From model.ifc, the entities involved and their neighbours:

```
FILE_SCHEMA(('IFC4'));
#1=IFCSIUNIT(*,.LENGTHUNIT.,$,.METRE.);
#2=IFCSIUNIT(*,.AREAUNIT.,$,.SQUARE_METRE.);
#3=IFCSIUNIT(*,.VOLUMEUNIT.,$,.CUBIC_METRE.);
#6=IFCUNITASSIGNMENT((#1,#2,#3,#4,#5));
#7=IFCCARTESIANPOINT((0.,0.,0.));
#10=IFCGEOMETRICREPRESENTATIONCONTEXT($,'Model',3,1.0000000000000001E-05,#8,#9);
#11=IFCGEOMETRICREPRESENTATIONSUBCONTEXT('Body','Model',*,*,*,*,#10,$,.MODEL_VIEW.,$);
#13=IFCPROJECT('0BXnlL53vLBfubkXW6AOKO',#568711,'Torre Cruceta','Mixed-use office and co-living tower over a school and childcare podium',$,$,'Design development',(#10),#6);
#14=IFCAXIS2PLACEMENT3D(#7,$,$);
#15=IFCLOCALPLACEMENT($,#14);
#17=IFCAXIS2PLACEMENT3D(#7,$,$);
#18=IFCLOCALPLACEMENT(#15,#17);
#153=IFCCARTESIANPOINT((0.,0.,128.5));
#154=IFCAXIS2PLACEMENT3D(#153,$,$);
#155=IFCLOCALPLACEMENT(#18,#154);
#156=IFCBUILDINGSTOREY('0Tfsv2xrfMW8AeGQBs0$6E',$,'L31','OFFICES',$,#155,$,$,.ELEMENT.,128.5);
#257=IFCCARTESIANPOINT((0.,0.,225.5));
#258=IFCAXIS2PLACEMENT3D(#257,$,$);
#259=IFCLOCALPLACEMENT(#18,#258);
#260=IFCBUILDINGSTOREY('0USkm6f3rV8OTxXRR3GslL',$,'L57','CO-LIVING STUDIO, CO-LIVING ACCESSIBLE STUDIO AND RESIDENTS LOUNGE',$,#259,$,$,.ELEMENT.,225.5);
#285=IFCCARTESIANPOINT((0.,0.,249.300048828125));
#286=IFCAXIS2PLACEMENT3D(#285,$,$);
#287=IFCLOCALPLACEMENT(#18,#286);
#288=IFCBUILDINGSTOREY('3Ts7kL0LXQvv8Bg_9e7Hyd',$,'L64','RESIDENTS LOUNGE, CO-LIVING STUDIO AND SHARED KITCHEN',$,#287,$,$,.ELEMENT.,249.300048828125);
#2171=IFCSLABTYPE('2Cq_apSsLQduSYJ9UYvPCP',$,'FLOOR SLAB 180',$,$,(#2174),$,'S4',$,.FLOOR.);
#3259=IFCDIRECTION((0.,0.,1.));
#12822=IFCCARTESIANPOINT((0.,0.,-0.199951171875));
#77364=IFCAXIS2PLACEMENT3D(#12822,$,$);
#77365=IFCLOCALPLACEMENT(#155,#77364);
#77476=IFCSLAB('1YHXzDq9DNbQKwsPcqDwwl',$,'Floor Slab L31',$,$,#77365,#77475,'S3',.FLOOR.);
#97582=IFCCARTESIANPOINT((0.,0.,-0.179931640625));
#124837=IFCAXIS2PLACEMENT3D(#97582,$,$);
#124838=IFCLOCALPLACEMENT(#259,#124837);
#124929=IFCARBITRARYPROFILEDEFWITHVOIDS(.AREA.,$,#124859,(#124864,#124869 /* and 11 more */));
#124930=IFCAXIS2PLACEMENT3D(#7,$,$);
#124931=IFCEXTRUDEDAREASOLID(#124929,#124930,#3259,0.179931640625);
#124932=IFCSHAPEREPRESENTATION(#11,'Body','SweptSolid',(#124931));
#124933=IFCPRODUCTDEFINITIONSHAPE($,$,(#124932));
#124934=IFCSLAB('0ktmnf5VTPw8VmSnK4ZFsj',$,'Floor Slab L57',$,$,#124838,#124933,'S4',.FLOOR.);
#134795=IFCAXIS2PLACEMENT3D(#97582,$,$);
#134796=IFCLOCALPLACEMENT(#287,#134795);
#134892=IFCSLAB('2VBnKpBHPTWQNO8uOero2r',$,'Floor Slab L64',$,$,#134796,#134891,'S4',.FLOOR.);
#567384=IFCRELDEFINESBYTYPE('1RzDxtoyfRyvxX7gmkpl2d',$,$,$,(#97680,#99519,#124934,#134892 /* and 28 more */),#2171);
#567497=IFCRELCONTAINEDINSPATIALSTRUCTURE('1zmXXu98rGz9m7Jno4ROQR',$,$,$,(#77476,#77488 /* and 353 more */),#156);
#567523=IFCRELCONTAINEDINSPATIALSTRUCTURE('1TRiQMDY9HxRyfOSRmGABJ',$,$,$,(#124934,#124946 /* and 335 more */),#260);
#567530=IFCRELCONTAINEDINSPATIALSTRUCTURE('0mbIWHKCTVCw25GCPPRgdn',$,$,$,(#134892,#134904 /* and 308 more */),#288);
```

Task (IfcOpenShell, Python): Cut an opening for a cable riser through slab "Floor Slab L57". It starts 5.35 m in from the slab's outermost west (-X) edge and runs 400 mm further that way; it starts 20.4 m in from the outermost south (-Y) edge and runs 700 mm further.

```python
import numpy as np
import ifcopenshell
import ifcopenshell.api.feature
import ifcopenshell.api.geometry
import ifcopenshell.api.root
import ifcopenshell.geom
import ifcopenshell.util.placement
import ifcopenshell.util.representation
import ifcopenshell.util.shape
import ifcopenshell.util.unit

model = ifcopenshell.open("model.ifc")
unit_scale = ifcopenshell.util.unit.calculate_unit_scale(model)
settings = ifcopenshell.geom.settings()


def volume(element):
    """Net volume in cubic metres, openings subtracted."""
    shape = ifcopenshell.geom.create_shape(settings, element)
    return ifcopenshell.util.shape.get_volume(shape.geometry)


slab = model.by_id(124934)
before = volume(slab)

# Extent in the slab's own axes, in metres. The edges named are its -X and -Y sides.
slab_shape = ifcopenshell.geom.create_shape(settings, slab)
vertices = ifcopenshell.util.shape.get_vertices(slab_shape.geometry)
x_min, y_min, bottom = vertices.min(axis=0)
top = vertices[:, 2].max()

opening = ifcopenshell.api.root.create_entity(model, ifc_class="IfcOpeningElement", name="Cable riser opening", predefined_type="OPENING")
context = ifcopenshell.util.representation.get_context(model, "Model", "Body", "MODEL_VIEW")
width, depth = 0.4, 0.7
outline = [(0.0, 0.0), (width, 0.0), (width, depth), (0.0, depth), (0.0, 0.0)]
# Overshoot both faces by 50 mm so the cut is clean.
shape = ifcopenshell.api.geometry.add_slab_representation(
    model, context=context, depth=top - bottom + 0.1, polyline=outline
)
ifcopenshell.api.geometry.assign_representation(model, product=opening, representation=shape)

matrix = ifcopenshell.util.placement.get_local_placement(slab.ObjectPlacement)
matrix[:, 3] = matrix @ np.append(np.array([x_min + 5.35, y_min + 20.4, bottom - 0.05]) / unit_scale, 1.0)
ifcopenshell.api.geometry.edit_object_placement(model, product=opening, matrix=matrix, is_si=False)
ifcopenshell.api.feature.add_feature(model, feature=opening, element=slab)

after = volume(slab)

print(f"slab volume {before:.3f} -> {after:.3f} m3")

model.write("model-out.ifc")
```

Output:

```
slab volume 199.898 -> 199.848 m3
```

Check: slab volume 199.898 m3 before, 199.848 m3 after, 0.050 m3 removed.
